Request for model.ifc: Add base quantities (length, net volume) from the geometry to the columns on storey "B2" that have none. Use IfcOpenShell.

First a look at what the model holds.

```python
import ifcopenshell
import ifcopenshell.util.element
import ifcopenshell.util.unit

model = ifcopenshell.open("model.ifc")
print(model.schema)
for unit_type in ("LENGTHUNIT", "AREAUNIT", "VOLUMEUNIT"):
    print(unit_type, ifcopenshell.util.unit.calculate_unit_scale(model, unit_type))
storey = next(s for s in model.by_type("IfcBuildingStorey") if s.Name == "B2")
columns = [e for e in ifcopenshell.util.element.get_decomposition(storey) if e.is_a("IfcColumn")]
for e in sorted(columns, key=lambda e: e.id()):
    print(e.id(), e.is_a(), e.Name, list(ifcopenshell.util.element.get_psets(e, qtos_only=True)), sep=" | ")
```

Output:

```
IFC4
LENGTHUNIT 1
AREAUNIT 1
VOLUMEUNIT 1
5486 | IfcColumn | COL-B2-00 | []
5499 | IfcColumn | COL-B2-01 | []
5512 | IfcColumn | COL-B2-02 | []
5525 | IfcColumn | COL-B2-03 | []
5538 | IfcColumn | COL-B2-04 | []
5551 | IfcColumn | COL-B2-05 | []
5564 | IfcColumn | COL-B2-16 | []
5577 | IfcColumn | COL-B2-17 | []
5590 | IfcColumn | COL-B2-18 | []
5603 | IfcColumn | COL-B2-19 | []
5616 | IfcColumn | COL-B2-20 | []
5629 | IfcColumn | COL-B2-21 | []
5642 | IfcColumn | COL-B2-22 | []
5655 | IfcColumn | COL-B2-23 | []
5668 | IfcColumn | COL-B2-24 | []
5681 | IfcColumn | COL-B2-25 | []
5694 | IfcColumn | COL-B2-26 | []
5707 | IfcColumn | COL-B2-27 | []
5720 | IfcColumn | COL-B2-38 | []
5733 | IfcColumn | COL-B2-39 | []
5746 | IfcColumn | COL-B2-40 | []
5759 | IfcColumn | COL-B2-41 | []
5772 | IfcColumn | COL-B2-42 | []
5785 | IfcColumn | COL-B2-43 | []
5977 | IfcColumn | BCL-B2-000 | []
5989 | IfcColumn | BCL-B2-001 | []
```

```python
import ifcopenshell
import ifcopenshell.api.pset
import ifcopenshell.geom
import ifcopenshell.util.element
import ifcopenshell.util.shape
import ifcopenshell.util.unit

model = ifcopenshell.open("model.ifc")
unit_scale = ifcopenshell.util.unit.calculate_unit_scale(model)
volume_scale = ifcopenshell.util.unit.calculate_unit_scale(model, "VOLUMEUNIT")
settings = ifcopenshell.geom.settings()

storey = next(s for s in model.by_type("IfcBuildingStorey") if s.Name == "B2")
columns = [e for e in ifcopenshell.util.element.get_decomposition(storey) if e.is_a("IfcColumn")]

for e in sorted(columns, key=lambda e: e.id()):
    if ifcopenshell.util.element.get_psets(e, qtos_only=True, should_inherit=False):
        continue
    # Geometry comes back in metres, in the element's own axes.
    shape = ifcopenshell.geom.create_shape(settings, e)
    values = {
        "Length": ifcopenshell.util.shape.get_z(shape.geometry) / unit_scale,
        "NetVolume": ifcopenshell.util.shape.get_volume(shape.geometry) / volume_scale,
    }
    qto = ifcopenshell.api.pset.add_qto(model, product=e, name="Qto_ColumnBaseQuantities")
    ifcopenshell.api.pset.edit_qto(model, qto=qto, properties=values)
    print(e.id(), {k: round(v, 3) for k, v in values.items()})

model.write("model_updated.ifc")
```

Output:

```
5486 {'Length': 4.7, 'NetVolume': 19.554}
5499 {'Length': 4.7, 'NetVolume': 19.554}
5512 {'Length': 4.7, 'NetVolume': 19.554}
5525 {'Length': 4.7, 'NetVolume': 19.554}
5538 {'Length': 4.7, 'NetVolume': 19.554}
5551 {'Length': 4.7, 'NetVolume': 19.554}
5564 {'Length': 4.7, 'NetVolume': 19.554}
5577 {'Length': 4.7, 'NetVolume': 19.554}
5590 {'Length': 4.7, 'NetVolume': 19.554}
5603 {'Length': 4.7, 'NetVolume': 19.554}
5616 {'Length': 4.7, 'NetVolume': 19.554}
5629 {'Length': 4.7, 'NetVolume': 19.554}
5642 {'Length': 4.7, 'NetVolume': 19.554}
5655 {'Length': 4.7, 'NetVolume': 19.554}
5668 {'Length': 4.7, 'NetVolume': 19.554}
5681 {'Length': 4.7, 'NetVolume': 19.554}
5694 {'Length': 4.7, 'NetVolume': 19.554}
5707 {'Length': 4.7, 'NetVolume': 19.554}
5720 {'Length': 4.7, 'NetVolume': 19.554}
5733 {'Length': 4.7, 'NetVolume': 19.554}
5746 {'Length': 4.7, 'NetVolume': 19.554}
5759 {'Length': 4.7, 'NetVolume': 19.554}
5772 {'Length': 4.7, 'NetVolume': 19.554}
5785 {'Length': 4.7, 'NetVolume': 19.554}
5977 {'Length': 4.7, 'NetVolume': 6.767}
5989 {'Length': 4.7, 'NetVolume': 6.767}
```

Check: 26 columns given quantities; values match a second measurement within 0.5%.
